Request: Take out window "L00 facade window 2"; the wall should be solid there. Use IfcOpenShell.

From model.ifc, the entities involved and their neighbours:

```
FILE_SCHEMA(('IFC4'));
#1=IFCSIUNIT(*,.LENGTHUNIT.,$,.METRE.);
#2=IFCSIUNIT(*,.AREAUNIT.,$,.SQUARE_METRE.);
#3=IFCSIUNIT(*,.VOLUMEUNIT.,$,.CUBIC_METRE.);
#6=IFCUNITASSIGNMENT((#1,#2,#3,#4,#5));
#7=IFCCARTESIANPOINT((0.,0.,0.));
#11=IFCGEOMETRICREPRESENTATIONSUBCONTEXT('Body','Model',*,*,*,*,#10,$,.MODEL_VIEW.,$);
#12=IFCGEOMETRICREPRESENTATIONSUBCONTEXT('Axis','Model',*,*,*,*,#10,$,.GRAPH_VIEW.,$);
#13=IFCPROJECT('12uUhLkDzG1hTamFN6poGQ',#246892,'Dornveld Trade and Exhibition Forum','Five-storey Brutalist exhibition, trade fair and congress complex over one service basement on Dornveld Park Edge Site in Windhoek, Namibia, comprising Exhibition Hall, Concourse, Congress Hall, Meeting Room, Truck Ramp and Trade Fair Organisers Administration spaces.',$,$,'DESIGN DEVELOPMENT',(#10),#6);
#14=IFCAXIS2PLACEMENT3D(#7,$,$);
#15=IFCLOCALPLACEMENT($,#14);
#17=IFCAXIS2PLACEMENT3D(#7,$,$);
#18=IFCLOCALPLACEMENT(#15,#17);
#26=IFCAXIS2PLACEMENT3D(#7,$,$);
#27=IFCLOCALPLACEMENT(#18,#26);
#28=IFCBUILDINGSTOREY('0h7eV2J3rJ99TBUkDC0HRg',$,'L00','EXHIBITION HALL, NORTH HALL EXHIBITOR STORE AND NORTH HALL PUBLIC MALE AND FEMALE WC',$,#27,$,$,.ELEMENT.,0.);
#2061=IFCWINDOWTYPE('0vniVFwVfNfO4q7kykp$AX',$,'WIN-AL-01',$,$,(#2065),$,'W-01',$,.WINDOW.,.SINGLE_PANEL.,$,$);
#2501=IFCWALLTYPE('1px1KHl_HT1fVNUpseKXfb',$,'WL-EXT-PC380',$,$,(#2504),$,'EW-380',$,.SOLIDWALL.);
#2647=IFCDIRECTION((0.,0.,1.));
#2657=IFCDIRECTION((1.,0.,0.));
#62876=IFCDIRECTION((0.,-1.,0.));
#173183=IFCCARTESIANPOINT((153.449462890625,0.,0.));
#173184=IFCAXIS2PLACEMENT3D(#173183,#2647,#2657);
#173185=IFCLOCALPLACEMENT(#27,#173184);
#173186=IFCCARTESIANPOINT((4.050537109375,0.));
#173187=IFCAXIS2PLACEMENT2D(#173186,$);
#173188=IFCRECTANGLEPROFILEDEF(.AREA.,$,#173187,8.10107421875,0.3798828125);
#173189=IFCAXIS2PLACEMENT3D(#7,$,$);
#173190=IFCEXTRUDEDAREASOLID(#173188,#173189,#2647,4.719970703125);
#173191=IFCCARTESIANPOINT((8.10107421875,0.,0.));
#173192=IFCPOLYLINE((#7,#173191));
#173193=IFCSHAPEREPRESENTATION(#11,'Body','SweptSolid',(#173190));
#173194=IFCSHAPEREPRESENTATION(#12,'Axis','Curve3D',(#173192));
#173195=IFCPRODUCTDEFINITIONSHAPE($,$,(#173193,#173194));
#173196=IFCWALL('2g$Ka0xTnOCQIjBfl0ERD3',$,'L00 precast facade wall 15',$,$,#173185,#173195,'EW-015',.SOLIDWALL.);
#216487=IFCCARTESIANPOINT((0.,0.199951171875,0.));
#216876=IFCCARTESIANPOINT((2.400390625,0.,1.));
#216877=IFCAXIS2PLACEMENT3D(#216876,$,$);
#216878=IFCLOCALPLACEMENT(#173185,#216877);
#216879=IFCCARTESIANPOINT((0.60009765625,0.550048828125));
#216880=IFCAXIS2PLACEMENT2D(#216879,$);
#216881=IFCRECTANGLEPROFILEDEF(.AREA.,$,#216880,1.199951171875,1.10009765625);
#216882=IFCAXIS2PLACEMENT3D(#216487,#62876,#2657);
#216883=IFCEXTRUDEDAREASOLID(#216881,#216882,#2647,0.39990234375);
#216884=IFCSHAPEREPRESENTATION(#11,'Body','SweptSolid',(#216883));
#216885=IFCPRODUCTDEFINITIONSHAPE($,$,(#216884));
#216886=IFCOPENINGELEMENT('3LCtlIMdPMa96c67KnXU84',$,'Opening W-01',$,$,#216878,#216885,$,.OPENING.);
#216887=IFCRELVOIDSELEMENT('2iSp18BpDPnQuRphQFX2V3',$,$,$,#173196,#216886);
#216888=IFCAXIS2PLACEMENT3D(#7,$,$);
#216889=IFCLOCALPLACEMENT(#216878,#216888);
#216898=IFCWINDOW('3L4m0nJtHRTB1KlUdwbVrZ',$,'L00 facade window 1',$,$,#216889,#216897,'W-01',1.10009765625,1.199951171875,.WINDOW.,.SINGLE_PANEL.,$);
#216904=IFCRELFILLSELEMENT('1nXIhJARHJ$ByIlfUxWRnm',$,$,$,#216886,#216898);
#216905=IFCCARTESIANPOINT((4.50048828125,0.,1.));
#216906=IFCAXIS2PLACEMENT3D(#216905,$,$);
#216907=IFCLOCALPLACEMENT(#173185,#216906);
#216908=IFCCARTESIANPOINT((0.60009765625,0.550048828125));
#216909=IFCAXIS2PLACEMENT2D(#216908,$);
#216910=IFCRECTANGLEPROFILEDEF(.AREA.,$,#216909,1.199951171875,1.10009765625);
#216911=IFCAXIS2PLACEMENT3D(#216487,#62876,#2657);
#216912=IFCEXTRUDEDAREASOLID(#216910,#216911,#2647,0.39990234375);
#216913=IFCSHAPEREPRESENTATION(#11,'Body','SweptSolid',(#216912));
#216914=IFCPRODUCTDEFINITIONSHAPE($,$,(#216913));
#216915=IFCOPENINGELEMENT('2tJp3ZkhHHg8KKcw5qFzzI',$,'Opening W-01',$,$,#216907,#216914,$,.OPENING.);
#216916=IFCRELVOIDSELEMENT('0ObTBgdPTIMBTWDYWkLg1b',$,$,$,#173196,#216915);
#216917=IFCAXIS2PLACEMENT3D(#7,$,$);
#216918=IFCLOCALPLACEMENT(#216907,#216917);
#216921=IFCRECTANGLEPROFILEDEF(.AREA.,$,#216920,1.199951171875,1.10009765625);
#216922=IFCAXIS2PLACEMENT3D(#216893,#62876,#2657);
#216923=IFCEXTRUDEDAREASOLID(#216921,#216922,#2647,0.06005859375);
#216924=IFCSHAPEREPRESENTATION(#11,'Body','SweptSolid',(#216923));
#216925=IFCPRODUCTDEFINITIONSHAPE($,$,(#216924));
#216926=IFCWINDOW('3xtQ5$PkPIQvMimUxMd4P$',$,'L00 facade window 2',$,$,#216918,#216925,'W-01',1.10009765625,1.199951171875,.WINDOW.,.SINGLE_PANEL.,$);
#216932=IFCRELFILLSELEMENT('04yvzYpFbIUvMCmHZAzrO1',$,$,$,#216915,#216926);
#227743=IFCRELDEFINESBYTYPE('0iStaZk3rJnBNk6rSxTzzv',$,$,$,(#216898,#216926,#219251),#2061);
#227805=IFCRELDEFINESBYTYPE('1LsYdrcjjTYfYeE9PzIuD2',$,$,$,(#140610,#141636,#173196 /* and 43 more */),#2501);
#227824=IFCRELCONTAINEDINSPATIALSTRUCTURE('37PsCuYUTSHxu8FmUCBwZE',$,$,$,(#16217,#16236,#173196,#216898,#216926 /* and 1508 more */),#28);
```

```python
import ifcopenshell
import ifcopenshell.api.feature
import ifcopenshell.api.root
import ifcopenshell.geom
import ifcopenshell.util.shape

model = ifcopenshell.open("model.ifc")
settings = ifcopenshell.geom.settings()


def volume(element):
    """Net volume in cubic metres, openings subtracted."""
    shape = ifcopenshell.geom.create_shape(settings, element)
    return ifcopenshell.util.shape.get_volume(shape.geometry)


window = model.by_id(216926)
opening = window.FillsVoids[0].RelatingOpeningElement
wall = opening.VoidsElements[0].RelatingBuildingElement
before = volume(wall)

ifcopenshell.api.root.remove_product(model, product=window)
ifcopenshell.api.feature.remove_feature(model, feature=opening)

after = volume(wall)

print(f"wall volume {before:.3f} -> {after:.3f} m3")

model.write("model_updated.ifc")
```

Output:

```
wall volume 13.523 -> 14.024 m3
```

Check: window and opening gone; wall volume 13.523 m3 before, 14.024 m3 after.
